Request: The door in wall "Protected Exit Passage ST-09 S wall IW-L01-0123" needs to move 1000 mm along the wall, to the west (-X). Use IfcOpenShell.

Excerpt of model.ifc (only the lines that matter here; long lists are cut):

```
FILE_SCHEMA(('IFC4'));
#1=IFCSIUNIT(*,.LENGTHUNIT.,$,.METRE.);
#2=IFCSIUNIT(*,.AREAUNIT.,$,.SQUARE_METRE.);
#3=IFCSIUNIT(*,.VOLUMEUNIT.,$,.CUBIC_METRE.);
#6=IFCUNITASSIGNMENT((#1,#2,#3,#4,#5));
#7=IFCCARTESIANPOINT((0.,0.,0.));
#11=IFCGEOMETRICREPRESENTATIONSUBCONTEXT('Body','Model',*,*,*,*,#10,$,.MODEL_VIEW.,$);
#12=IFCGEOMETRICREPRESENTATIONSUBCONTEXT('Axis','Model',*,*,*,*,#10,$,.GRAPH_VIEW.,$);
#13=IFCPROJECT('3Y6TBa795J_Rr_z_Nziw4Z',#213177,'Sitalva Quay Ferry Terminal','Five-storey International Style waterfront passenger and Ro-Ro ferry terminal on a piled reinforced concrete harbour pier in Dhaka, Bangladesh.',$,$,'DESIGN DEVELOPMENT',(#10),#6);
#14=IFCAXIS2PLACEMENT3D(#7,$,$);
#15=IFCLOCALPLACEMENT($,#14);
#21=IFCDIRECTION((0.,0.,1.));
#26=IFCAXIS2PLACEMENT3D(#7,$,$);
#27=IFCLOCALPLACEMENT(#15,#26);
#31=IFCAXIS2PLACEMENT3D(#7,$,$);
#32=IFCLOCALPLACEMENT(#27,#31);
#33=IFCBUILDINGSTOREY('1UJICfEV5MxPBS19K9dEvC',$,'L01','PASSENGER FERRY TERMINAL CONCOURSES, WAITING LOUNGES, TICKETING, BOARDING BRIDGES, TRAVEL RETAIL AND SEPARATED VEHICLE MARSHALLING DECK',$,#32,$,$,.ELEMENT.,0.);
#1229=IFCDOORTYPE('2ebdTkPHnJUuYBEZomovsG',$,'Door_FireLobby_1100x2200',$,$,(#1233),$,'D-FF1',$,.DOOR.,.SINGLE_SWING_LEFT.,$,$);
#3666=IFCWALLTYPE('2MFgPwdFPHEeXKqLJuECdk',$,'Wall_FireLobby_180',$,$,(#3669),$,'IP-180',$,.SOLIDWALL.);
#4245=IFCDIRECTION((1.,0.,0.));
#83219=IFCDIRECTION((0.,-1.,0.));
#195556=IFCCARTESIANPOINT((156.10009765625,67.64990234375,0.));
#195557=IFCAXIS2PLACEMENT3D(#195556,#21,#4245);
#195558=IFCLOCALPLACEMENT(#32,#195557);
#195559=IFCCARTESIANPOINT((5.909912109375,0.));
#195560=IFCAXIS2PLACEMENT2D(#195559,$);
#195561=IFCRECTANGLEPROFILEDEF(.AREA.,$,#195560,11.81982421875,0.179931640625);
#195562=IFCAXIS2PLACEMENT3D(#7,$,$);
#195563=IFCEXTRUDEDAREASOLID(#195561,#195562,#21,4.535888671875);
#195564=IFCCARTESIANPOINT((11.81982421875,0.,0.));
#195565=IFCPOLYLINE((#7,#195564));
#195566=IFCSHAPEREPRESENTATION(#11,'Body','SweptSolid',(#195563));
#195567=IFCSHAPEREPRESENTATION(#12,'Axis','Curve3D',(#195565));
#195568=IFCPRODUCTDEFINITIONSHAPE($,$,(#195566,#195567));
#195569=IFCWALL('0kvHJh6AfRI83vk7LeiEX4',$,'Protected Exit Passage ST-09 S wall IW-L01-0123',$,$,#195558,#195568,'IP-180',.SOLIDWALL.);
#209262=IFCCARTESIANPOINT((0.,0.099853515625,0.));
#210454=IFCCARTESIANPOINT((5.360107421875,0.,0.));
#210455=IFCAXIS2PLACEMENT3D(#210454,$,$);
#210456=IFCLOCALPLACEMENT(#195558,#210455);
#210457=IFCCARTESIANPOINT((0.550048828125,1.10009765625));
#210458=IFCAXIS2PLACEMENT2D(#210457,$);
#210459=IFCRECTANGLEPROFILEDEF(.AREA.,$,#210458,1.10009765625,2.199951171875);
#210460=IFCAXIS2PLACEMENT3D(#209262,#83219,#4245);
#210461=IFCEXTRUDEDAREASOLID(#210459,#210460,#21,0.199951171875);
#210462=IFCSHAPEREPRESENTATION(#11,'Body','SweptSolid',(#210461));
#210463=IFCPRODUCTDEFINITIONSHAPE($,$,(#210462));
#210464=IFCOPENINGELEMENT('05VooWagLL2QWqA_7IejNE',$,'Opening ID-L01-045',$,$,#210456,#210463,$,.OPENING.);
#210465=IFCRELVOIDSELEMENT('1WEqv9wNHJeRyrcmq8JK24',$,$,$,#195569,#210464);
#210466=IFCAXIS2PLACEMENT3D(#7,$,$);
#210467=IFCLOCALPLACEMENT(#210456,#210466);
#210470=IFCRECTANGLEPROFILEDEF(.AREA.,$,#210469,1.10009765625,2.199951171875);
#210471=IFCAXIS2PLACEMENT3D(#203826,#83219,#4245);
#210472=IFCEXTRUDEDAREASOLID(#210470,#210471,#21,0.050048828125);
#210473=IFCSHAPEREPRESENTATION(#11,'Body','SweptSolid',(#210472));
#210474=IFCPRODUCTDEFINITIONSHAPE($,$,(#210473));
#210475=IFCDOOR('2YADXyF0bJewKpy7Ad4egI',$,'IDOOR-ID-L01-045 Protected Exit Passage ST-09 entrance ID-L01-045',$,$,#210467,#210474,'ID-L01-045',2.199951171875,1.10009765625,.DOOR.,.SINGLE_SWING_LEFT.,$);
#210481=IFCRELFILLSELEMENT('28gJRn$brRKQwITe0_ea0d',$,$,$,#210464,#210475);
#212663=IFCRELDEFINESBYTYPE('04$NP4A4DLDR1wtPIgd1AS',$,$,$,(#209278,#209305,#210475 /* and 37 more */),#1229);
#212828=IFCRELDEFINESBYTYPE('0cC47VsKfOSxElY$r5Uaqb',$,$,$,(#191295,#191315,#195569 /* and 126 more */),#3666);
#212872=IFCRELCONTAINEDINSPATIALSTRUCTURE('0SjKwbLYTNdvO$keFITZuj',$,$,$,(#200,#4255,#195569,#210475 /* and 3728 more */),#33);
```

```python
import ifcopenshell
import ifcopenshell.api.geometry
import ifcopenshell.util.placement
import ifcopenshell.util.unit

model = ifcopenshell.open("model.ifc")
unit_scale = ifcopenshell.util.unit.calculate_unit_scale(model)

door = model.by_id(210475)
opening = door.FillsVoids[0].RelatingOpeningElement
wall = opening.VoidsElements[0].RelatingBuildingElement

wall_matrix = ifcopenshell.util.placement.get_local_placement(wall.ObjectPlacement)
shift = wall_matrix[:3, 0] * -1 / unit_scale
before = ifcopenshell.util.placement.get_local_placement(door.ObjectPlacement)[:3, 3].copy()

# The door is placed relative to its opening, so it follows when the opening moves.
matrix = ifcopenshell.util.placement.get_local_placement(opening.ObjectPlacement)
matrix[:3, 3] += shift
ifcopenshell.api.geometry.edit_object_placement(
    model, product=opening, matrix=matrix, is_si=False, should_transform_children=True
)

after = ifcopenshell.util.placement.get_local_placement(door.ObjectPlacement)[:3, 3]
print("door moved by", (after - before).round(3) + 0.0)

model.write("model_updated.ifc")
```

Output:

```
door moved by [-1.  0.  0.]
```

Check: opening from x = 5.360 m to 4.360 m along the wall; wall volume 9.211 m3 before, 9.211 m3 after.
